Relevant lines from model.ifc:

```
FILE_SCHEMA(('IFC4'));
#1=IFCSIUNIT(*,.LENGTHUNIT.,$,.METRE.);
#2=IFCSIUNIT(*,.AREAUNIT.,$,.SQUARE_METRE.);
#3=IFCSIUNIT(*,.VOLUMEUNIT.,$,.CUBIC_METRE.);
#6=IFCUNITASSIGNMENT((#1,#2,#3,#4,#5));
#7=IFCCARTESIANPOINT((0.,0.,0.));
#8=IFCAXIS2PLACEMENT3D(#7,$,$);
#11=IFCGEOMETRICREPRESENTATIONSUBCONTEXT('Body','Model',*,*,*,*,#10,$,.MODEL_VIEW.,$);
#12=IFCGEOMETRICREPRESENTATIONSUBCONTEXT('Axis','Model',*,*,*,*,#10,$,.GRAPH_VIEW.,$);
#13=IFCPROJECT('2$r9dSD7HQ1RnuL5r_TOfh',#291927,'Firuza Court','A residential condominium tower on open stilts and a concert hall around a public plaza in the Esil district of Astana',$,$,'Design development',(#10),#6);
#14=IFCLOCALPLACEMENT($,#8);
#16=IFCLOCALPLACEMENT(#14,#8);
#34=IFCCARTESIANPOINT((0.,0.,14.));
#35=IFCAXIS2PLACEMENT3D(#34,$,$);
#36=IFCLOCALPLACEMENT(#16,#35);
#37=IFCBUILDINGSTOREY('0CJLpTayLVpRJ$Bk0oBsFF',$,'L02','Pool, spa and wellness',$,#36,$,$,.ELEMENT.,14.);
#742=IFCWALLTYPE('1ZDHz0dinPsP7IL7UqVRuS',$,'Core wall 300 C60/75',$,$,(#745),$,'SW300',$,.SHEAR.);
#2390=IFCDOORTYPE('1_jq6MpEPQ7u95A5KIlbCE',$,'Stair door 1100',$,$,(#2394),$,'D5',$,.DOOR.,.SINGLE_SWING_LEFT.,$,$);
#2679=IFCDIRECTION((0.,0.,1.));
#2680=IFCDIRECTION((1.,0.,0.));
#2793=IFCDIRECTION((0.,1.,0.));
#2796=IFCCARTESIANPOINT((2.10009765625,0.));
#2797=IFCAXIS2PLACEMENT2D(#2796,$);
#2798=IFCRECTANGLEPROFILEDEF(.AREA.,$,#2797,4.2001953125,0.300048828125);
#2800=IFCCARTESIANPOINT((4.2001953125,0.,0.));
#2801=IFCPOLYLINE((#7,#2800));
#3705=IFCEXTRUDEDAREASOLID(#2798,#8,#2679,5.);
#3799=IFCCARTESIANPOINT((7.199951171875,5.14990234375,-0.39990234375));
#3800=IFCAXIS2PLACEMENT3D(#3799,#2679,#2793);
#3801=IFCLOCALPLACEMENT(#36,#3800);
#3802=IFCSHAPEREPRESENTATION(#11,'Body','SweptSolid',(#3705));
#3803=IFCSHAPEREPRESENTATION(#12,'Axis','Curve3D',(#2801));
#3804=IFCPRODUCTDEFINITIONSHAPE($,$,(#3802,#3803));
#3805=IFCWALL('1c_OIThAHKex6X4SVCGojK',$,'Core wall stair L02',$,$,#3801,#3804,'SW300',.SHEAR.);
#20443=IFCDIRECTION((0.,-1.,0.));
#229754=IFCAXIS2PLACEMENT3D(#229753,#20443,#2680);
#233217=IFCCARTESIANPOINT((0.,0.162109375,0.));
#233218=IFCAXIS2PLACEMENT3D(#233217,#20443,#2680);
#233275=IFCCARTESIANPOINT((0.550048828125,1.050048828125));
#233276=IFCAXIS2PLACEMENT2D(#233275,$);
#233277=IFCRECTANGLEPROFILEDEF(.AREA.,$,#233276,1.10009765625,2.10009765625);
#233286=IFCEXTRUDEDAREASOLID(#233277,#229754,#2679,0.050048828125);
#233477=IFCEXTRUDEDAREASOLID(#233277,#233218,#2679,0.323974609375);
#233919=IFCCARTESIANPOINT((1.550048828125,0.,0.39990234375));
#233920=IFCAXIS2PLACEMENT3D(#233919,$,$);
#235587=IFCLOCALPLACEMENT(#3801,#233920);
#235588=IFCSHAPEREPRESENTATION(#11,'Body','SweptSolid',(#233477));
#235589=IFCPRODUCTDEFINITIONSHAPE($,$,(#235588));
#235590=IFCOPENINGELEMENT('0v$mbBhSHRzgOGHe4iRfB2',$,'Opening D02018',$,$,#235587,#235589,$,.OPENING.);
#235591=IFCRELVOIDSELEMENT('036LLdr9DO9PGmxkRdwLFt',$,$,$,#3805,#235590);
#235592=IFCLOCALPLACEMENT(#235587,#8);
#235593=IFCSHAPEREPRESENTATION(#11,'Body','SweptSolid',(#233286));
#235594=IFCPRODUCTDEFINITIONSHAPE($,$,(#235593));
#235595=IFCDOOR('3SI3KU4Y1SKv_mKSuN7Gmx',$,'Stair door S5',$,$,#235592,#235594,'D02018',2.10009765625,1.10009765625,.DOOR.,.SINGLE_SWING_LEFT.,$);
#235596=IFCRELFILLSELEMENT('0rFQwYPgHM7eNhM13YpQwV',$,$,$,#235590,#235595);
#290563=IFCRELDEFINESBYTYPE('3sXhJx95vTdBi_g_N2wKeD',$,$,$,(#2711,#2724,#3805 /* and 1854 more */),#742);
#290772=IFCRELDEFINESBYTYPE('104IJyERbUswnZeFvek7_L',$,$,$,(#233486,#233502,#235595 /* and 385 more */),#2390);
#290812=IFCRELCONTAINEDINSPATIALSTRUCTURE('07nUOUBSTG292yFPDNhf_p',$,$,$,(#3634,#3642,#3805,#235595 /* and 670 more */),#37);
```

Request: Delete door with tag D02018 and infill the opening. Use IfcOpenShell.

```python
import ifcopenshell
import ifcopenshell.api.feature
import ifcopenshell.api.root
import ifcopenshell.geom
import ifcopenshell.util.shape

model = ifcopenshell.open("model.ifc")
settings = ifcopenshell.geom.settings()


def volume(element):
    """Net volume in cubic metres, openings subtracted."""
    shape = ifcopenshell.geom.create_shape(settings, element)
    return ifcopenshell.util.shape.get_volume(shape.geometry)


door = model.by_guid("3SI3KU4Y1SKv_mKSuN7Gmx")
opening = door.FillsVoids[0].RelatingOpeningElement
wall = opening.VoidsElements[0].RelatingBuildingElement
before = volume(wall)

ifcopenshell.api.root.remove_product(model, product=door)
ifcopenshell.api.feature.remove_feature(model, feature=opening)

after = volume(wall)

print(f"wall volume {before:.3f} -> {after:.3f} m3")

model.write("model_v2.ifc")
```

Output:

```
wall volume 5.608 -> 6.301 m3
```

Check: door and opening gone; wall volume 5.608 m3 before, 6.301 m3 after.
